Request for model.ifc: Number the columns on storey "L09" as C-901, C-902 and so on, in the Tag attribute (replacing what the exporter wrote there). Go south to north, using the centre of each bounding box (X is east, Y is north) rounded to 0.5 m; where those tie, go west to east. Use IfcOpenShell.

First a look at what the model holds.

```python
import ifcopenshell
import ifcopenshell.util.element
import ifcopenshell.util.placement

model = ifcopenshell.open("model.ifc")
print(model.schema)
storey = next(s for s in model.by_type("IfcBuildingStorey") if s.Name == "L09")
columns = [e for e in ifcopenshell.util.element.get_decomposition(storey) if e.is_a("IfcColumn")]
for e in sorted(columns, key=lambda e: e.id()):
    origin = ifcopenshell.util.placement.get_local_placement(e.ObjectPlacement)[:3, 3]
    print(e.id(), e.Tag, e.Name, origin.round(2) + 0.0, sep=" | ")
```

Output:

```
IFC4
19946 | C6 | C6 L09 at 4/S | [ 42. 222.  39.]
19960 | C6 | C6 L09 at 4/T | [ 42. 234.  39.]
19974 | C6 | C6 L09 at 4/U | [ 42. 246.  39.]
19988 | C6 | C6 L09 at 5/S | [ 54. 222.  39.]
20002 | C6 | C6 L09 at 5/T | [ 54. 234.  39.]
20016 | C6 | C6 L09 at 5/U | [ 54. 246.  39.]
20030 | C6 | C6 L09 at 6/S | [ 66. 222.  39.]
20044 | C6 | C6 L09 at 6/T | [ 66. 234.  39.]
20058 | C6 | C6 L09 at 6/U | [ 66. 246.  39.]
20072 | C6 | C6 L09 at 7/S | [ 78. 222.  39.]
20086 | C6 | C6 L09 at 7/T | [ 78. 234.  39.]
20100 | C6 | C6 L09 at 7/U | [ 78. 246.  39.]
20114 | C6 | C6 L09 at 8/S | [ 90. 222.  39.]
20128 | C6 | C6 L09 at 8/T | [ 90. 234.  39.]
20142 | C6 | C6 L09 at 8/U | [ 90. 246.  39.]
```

```python
import ifcopenshell
import ifcopenshell.geom
import ifcopenshell.util.element
import ifcopenshell.util.shape

model = ifcopenshell.open("model.ifc")
settings = ifcopenshell.geom.settings()
settings.set("use-world-coords", True)


def centre(element):
    shape = ifcopenshell.geom.create_shape(settings, element)
    return ifcopenshell.util.shape.get_bbox_centroid(shape.geometry)


storey = next(s for s in model.by_type("IfcBuildingStorey") if s.Name == "L09")
columns = [e for e in ifcopenshell.util.element.get_decomposition(storey) if e.is_a("IfcColumn")]

# Insertion points can sit at a corner or the storey origin, so sort by the geometry (in metres).
centres = {e: centre(e) for e in columns}
columns.sort(key=lambda e: (round(centres[e][1] / 0.5), centres[e][0]))

for i, e in enumerate(columns, start=1):
    number = f"C-9{i:02d}"
    e.Tag = number
    print(e.id(), number)

model.write("model_rev.ifc")
```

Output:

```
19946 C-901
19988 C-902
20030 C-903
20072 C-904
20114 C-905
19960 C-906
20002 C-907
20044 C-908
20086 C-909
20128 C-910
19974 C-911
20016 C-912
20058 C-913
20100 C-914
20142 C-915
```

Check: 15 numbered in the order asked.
